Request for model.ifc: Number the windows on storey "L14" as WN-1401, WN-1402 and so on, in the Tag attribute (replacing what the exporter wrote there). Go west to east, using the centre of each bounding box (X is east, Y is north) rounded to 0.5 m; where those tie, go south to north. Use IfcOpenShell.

First a look at what the model holds.

```python
import ifcopenshell
import ifcopenshell.util.element
import ifcopenshell.util.placement

model = ifcopenshell.open("model.ifc")
print(model.schema)
storey = next(s for s in model.by_type("IfcBuildingStorey") if s.Name == "L14")
windows = [e for e in ifcopenshell.util.element.get_decomposition(storey) if e.is_a("IfcWindow")]
for e in sorted(windows, key=lambda e: e.id()):
    origin = ifcopenshell.util.placement.get_local_placement(e.ObjectPlacement)[:3, 3]
    print(e.id(), e.Tag, e.Name, origin.round(2) + 0.0, sep=" | ")
```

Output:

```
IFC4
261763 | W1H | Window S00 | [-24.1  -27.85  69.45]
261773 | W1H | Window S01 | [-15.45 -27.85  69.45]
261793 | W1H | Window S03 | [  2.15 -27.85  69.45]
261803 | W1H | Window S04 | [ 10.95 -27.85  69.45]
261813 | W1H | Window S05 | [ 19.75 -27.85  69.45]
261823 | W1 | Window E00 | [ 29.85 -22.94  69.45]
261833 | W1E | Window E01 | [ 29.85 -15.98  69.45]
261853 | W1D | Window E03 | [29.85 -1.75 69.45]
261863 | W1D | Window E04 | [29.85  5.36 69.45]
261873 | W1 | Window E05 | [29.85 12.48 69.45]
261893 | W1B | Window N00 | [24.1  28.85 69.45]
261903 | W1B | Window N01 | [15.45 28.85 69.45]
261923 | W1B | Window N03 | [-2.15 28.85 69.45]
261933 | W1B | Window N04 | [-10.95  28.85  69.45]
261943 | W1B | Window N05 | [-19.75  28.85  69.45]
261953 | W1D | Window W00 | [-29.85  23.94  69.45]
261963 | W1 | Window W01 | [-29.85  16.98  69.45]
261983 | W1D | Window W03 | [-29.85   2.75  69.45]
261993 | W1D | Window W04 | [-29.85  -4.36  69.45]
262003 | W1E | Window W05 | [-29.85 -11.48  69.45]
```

```python
import ifcopenshell
import ifcopenshell.geom
import ifcopenshell.util.element
import ifcopenshell.util.shape

model = ifcopenshell.open("model.ifc")
settings = ifcopenshell.geom.settings()
settings.set("use-world-coords", True)


def centre(element):
    shape = ifcopenshell.geom.create_shape(settings, element)
    return ifcopenshell.util.shape.get_bbox_centroid(shape.geometry)


storey = next(s for s in model.by_type("IfcBuildingStorey") if s.Name == "L14")
windows = [e for e in ifcopenshell.util.element.get_decomposition(storey) if e.is_a("IfcWindow")]

# Insertion points can sit at a corner or the storey origin, so sort by the geometry (in metres).
centres = {e: centre(e) for e in windows}
windows.sort(key=lambda e: (round(centres[e][0] / 0.5), centres[e][1]))

for i, e in enumerate(windows, start=1):
    number = f"WN-14{i:02d}"
    e.Tag = number
    print(e.id(), number)

model.write("model_rev.ifc")
```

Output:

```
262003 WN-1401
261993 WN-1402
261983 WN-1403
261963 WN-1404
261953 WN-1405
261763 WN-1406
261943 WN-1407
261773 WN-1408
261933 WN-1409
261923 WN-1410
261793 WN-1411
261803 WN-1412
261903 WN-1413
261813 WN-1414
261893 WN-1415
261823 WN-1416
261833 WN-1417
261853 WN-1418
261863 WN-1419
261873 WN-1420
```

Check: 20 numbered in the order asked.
